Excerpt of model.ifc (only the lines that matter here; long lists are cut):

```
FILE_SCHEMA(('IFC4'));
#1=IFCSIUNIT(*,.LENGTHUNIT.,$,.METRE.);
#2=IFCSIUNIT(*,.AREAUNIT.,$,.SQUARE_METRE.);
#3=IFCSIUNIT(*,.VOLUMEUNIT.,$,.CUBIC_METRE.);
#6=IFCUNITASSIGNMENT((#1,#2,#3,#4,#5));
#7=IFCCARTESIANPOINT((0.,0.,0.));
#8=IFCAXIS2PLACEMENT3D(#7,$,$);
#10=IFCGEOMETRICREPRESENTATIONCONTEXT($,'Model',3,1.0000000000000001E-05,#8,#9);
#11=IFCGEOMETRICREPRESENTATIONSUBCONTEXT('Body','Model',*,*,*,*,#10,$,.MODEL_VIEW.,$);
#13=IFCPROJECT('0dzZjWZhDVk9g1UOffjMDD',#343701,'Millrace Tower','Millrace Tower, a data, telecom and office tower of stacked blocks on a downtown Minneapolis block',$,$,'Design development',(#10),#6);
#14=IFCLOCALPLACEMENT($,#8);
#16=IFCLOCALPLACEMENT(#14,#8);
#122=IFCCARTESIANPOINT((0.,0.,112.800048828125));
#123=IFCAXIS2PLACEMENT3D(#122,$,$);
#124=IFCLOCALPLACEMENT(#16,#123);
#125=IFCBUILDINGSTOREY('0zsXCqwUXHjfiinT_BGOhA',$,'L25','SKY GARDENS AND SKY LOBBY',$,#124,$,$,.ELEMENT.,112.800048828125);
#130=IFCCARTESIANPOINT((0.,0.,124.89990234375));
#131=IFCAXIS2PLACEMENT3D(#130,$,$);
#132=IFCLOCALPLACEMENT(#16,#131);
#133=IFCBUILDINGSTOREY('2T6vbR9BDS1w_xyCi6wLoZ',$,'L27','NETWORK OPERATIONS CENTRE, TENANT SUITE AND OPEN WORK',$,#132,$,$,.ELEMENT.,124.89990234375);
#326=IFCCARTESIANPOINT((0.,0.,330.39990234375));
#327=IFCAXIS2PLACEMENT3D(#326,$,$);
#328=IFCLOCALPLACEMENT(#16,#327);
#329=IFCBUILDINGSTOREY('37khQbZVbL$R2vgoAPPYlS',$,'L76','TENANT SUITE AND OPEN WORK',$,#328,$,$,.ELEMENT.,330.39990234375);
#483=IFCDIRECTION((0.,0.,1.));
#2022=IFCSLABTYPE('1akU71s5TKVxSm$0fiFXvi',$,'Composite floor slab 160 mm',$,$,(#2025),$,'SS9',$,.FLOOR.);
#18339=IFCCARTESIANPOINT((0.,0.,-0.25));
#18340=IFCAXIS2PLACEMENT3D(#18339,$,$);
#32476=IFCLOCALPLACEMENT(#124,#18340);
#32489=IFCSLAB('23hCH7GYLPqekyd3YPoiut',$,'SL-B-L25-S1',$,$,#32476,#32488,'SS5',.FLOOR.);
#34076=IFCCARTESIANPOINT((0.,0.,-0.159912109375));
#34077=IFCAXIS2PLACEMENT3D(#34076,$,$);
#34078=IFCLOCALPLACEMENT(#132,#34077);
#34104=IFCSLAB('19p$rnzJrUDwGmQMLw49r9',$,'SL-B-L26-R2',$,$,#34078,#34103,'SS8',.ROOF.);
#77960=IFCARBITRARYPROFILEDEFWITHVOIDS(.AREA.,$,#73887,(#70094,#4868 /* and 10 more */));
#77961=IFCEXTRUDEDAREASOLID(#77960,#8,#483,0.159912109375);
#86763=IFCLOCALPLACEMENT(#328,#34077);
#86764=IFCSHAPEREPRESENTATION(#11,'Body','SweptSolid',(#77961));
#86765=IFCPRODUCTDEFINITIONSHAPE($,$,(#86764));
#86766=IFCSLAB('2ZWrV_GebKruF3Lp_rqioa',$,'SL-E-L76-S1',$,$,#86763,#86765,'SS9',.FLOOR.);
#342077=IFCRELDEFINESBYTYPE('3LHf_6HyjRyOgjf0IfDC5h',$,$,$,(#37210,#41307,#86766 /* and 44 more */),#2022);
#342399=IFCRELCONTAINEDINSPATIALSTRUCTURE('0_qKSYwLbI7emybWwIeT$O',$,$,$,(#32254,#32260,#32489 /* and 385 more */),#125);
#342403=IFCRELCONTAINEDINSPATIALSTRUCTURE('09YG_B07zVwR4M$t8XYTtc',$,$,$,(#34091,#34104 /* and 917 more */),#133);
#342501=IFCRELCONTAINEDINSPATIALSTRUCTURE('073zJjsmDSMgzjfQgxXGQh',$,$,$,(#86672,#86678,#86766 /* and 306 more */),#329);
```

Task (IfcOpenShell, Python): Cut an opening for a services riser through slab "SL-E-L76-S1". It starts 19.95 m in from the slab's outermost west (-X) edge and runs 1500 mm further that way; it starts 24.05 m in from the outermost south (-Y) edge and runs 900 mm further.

```python
import numpy as np
import ifcopenshell
import ifcopenshell.api.feature
import ifcopenshell.api.geometry
import ifcopenshell.api.root
import ifcopenshell.geom
import ifcopenshell.util.placement
import ifcopenshell.util.representation
import ifcopenshell.util.shape
import ifcopenshell.util.unit

model = ifcopenshell.open("model.ifc")
unit_scale = ifcopenshell.util.unit.calculate_unit_scale(model)
settings = ifcopenshell.geom.settings()


def volume(element):
    """Net volume in cubic metres, openings subtracted."""
    shape = ifcopenshell.geom.create_shape(settings, element)
    return ifcopenshell.util.shape.get_volume(shape.geometry)


slab = model.by_guid("2ZWrV_GebKruF3Lp_rqioa")
before = volume(slab)

# Extent in the slab's own axes, in metres. The edges named are its -X and -Y sides.
slab_shape = ifcopenshell.geom.create_shape(settings, slab)
vertices = ifcopenshell.util.shape.get_vertices(slab_shape.geometry)
x_min, y_min, bottom = vertices.min(axis=0)
top = vertices[:, 2].max()

opening = ifcopenshell.api.root.create_entity(model, ifc_class="IfcOpeningElement", name="Services riser opening", predefined_type="OPENING")
context = ifcopenshell.util.representation.get_context(model, "Model", "Body", "MODEL_VIEW")
width, depth = 1.5, 0.9
outline = [(0.0, 0.0), (width, 0.0), (width, depth), (0.0, depth), (0.0, 0.0)]
# Overshoot both faces by 50 mm so the cut is clean.
shape = ifcopenshell.api.geometry.add_slab_representation(
    model, context=context, depth=top - bottom + 0.1, polyline=outline
)
ifcopenshell.api.geometry.assign_representation(model, product=opening, representation=shape)

matrix = ifcopenshell.util.placement.get_local_placement(slab.ObjectPlacement)
matrix[:, 3] = matrix @ np.append(np.array([x_min + 19.95, y_min + 24.05, bottom - 0.05]) / unit_scale, 1.0)
ifcopenshell.api.geometry.edit_object_placement(model, product=opening, matrix=matrix, is_si=False)
ifcopenshell.api.feature.add_feature(model, feature=opening, element=slab)

after = volume(slab)

print(f"slab volume {before:.3f} -> {after:.3f} m3")

model.write("model-out.ifc")
```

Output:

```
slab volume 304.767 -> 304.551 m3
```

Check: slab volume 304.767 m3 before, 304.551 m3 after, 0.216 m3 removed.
